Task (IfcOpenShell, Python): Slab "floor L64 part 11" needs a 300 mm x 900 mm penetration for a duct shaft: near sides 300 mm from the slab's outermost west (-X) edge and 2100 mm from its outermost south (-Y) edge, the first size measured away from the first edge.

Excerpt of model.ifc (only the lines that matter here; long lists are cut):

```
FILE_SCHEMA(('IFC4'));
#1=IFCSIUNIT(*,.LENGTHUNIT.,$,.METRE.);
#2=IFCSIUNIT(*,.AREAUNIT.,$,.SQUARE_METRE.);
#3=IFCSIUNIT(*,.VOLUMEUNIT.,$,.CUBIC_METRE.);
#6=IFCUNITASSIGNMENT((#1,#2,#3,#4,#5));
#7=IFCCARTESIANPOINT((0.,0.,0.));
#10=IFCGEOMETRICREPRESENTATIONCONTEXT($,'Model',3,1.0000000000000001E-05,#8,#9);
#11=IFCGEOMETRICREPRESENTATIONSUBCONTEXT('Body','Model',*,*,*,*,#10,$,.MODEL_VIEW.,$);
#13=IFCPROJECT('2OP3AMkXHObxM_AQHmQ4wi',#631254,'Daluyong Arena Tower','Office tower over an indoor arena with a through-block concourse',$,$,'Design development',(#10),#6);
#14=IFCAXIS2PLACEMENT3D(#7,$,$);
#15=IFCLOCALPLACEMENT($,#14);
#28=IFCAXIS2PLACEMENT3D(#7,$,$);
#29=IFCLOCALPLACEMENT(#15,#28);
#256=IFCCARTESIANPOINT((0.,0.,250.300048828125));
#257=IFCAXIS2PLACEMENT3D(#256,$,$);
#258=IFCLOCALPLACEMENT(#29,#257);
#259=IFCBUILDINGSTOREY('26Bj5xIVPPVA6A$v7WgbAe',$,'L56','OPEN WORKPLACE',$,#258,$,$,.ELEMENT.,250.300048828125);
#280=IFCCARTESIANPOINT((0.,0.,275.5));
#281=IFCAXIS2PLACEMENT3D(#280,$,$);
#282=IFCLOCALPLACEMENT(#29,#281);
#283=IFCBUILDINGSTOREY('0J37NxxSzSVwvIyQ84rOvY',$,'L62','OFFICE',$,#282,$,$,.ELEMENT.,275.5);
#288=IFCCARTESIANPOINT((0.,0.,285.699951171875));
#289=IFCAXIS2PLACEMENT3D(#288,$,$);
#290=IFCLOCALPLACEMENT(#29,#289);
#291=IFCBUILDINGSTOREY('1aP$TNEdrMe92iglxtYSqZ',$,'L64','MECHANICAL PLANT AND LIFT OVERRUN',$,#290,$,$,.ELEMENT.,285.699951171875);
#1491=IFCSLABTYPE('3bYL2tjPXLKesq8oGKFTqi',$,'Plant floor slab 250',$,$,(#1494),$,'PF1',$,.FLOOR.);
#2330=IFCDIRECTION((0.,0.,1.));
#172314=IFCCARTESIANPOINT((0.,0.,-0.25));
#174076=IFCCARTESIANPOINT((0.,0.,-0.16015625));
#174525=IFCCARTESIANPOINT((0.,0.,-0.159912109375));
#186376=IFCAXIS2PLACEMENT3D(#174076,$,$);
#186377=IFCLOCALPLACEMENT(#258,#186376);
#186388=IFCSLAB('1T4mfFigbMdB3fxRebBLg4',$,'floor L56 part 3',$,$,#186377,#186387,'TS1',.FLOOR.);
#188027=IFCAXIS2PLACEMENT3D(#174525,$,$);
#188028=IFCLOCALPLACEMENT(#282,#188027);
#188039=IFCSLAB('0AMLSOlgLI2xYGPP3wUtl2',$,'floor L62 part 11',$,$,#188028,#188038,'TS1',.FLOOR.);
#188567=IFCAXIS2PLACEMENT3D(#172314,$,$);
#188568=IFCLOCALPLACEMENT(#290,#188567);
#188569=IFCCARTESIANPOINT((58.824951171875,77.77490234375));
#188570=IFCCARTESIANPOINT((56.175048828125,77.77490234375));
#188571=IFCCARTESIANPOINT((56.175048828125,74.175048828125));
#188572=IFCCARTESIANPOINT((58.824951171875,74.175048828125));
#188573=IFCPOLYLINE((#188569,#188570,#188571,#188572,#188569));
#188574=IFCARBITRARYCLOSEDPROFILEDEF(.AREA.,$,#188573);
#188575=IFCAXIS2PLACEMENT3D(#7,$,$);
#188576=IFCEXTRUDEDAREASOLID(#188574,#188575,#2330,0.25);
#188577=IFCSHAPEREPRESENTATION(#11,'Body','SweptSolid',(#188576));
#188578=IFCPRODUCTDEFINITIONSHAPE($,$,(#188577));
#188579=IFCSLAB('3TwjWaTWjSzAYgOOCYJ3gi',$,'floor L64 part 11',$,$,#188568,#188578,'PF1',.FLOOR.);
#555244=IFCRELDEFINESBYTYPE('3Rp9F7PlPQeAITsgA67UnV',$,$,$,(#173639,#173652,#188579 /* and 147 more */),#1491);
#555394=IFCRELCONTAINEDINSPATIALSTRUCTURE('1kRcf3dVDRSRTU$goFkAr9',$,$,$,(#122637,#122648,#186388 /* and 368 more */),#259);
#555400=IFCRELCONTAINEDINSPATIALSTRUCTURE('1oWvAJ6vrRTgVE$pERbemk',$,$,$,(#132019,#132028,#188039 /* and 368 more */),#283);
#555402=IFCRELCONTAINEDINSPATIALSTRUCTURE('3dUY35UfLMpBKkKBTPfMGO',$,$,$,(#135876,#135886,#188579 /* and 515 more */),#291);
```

```python
import numpy as np
import ifcopenshell
import ifcopenshell.api.feature
import ifcopenshell.api.geometry
import ifcopenshell.api.root
import ifcopenshell.geom
import ifcopenshell.util.placement
import ifcopenshell.util.representation
import ifcopenshell.util.shape
import ifcopenshell.util.unit

model = ifcopenshell.open("model.ifc")
unit_scale = ifcopenshell.util.unit.calculate_unit_scale(model)
settings = ifcopenshell.geom.settings()


def volume(element):
    """Net volume in cubic metres, openings subtracted."""
    shape = ifcopenshell.geom.create_shape(settings, element)
    return ifcopenshell.util.shape.get_volume(shape.geometry)


slab = model.by_guid("3TwjWaTWjSzAYgOOCYJ3gi")
before = volume(slab)

# Extent in the slab's own axes, in metres. The edges named are its -X and -Y sides.
slab_shape = ifcopenshell.geom.create_shape(settings, slab)
vertices = ifcopenshell.util.shape.get_vertices(slab_shape.geometry)
x_min, y_min, bottom = vertices.min(axis=0)
top = vertices[:, 2].max()

opening = ifcopenshell.api.root.create_entity(model, ifc_class="IfcOpeningElement", name="Duct shaft opening", predefined_type="OPENING")
context = ifcopenshell.util.representation.get_context(model, "Model", "Body", "MODEL_VIEW")
width, depth = 0.3, 0.9
outline = [(0.0, 0.0), (width, 0.0), (width, depth), (0.0, depth), (0.0, 0.0)]
# Overshoot both faces by 50 mm so the cut is clean.
shape = ifcopenshell.api.geometry.add_slab_representation(
    model, context=context, depth=top - bottom + 0.1, polyline=outline
)
ifcopenshell.api.geometry.assign_representation(model, product=opening, representation=shape)

matrix = ifcopenshell.util.placement.get_local_placement(slab.ObjectPlacement)
matrix[:, 3] = matrix @ np.append(np.array([x_min + 0.3, y_min + 2.1, bottom - 0.05]) / unit_scale, 1.0)
ifcopenshell.api.geometry.edit_object_placement(model, product=opening, matrix=matrix, is_si=False)
ifcopenshell.api.feature.add_feature(model, feature=opening, element=slab)

after = volume(slab)

print(f"slab volume {before:.3f} -> {after:.3f} m3")

model.write("model_edited.ifc")
```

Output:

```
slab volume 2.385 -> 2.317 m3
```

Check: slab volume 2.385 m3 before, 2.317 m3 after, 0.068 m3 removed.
